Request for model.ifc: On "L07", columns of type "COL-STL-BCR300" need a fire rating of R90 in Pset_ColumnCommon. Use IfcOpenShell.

First a look at what the model holds.

```python
import ifcopenshell
import ifcopenshell.util.element

model = ifcopenshell.open("model.ifc")
print(model.schema)
storey = next(s for s in model.by_type("IfcBuildingStorey") if s.Name == "L07")
columns = [e for e in ifcopenshell.util.element.get_decomposition(storey) if e.is_a("IfcColumn")]
seen = {}
for e in columns:
    element_type = ifcopenshell.util.element.get_type(e)
    key = (element_type.Name if element_type != e and element_type else None, ifcopenshell.util.element.get_pset(e, "Pset_ColumnCommon", "FireRating"))
    seen[key] = seen.get(key, 0) + 1
for (name, value), count in sorted(seen.items(), key=str):
    print(count, "x", name, "|", value)
```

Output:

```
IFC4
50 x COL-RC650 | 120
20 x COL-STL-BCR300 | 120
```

```python
import ifcopenshell
import ifcopenshell.api.pset
import ifcopenshell.util.element

model = ifcopenshell.open("model.ifc")

storey = next(s for s in model.by_type("IfcBuildingStorey") if s.Name == "L07")
columns = [e for e in ifcopenshell.util.element.get_decomposition(storey) if e.is_a("IfcColumn")]

count = 0
for e in columns:
    element_type = ifcopenshell.util.element.get_type(e)
    if element_type in (None, e) or element_type.Name != "COL-STL-BCR300":
        continue
    # add_pset returns the element's existing set when there is one.
    pset = ifcopenshell.api.pset.add_pset(model, product=e, name="Pset_ColumnCommon")
    ifcopenshell.api.pset.edit_pset(model, pset=pset, properties={"FireRating": "R90"})
    count += 1

print(count, "columns updated")

model.write("model-out.ifc")
```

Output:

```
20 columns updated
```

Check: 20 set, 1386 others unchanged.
